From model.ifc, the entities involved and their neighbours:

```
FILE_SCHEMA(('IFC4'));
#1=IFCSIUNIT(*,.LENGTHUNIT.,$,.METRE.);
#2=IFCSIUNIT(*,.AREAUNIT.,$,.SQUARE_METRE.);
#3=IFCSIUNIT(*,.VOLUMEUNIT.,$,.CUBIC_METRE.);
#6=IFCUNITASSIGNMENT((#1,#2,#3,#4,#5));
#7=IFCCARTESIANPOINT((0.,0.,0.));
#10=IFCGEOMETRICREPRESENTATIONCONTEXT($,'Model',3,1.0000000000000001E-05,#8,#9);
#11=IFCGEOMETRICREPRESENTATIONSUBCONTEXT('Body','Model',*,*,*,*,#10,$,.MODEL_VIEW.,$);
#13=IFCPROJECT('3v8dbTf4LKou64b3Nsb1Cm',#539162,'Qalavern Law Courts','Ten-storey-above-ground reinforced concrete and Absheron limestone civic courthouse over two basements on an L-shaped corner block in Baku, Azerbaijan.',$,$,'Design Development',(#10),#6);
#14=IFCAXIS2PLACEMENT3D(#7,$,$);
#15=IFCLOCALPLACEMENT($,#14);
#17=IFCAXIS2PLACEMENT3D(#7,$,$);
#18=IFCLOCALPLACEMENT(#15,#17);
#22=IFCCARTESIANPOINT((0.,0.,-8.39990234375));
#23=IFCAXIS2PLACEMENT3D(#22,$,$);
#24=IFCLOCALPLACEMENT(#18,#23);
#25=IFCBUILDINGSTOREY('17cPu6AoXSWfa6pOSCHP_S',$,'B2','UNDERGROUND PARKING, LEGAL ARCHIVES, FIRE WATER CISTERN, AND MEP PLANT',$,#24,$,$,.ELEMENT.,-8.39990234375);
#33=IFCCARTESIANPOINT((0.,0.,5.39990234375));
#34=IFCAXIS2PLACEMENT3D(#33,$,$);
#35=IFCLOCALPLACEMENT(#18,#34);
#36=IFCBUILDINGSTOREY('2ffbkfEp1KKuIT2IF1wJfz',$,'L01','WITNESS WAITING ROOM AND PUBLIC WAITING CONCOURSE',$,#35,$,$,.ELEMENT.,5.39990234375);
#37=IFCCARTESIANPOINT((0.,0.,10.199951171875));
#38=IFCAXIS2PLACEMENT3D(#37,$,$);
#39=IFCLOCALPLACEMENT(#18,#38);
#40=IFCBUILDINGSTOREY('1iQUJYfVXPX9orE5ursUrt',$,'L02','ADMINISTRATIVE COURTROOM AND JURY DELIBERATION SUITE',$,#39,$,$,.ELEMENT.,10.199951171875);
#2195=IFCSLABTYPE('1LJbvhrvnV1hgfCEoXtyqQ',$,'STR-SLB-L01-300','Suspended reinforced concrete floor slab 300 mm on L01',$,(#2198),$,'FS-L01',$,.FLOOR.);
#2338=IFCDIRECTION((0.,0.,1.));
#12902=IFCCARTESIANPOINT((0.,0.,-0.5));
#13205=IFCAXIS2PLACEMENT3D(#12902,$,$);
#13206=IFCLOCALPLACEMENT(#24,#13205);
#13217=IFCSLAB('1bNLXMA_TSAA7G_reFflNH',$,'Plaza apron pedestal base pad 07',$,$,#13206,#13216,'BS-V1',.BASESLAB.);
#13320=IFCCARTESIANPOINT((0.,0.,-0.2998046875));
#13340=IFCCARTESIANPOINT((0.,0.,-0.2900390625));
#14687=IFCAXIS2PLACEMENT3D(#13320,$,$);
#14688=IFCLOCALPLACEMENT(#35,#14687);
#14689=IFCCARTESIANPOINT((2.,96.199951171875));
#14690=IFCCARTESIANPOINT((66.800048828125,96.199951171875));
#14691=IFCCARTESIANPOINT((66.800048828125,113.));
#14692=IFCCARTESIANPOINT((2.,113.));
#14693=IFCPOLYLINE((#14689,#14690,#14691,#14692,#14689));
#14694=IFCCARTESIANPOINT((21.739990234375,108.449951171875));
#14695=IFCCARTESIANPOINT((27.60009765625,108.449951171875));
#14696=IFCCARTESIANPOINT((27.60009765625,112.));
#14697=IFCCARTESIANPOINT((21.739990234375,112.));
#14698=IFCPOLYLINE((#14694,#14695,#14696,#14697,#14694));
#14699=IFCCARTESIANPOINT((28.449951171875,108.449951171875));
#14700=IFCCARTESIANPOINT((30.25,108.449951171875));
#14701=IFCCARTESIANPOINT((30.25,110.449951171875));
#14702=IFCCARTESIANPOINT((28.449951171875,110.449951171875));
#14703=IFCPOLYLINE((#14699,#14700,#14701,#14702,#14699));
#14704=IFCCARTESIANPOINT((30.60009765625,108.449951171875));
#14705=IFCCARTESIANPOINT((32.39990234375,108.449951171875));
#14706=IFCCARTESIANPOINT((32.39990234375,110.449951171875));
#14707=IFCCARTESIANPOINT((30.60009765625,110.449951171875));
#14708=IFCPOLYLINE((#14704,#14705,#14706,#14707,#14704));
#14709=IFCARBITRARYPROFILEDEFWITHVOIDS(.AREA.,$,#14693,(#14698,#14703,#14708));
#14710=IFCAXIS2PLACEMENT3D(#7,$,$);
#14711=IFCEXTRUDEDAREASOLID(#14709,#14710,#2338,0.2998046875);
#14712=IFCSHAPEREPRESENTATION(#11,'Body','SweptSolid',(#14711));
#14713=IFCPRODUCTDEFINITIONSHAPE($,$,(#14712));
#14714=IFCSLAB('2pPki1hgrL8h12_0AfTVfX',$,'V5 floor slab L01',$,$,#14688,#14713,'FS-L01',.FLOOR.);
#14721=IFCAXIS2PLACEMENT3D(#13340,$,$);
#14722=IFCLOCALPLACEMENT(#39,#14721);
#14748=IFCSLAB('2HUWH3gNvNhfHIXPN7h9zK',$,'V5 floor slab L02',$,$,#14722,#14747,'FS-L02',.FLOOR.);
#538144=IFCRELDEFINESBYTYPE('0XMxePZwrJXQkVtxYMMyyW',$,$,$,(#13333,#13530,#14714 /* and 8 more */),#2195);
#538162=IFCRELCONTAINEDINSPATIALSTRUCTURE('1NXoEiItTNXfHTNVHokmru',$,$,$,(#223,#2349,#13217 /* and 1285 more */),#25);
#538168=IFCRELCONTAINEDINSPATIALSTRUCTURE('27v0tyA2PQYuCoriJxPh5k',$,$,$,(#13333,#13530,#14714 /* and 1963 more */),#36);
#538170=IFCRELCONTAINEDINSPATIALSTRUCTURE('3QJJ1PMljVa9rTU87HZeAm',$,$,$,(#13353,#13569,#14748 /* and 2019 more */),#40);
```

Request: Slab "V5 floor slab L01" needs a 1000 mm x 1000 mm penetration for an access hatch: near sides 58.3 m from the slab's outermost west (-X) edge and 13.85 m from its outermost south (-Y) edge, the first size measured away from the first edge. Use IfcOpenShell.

```python
import numpy as np
import ifcopenshell
import ifcopenshell.api.feature
import ifcopenshell.api.geometry
import ifcopenshell.api.root
import ifcopenshell.geom
import ifcopenshell.util.placement
import ifcopenshell.util.representation
import ifcopenshell.util.shape
import ifcopenshell.util.unit

model = ifcopenshell.open("model.ifc")
unit_scale = ifcopenshell.util.unit.calculate_unit_scale(model)
settings = ifcopenshell.geom.settings()


def volume(element):
    """Net volume in cubic metres, openings subtracted."""
    shape = ifcopenshell.geom.create_shape(settings, element)
    return ifcopenshell.util.shape.get_volume(shape.geometry)


slab = model.by_guid("2pPki1hgrL8h12_0AfTVfX")
before = volume(slab)

# Extent in the slab's own axes, in metres. The edges named are its -X and -Y sides.
slab_shape = ifcopenshell.geom.create_shape(settings, slab)
vertices = ifcopenshell.util.shape.get_vertices(slab_shape.geometry)
x_min, y_min, bottom = vertices.min(axis=0)
top = vertices[:, 2].max()

opening = ifcopenshell.api.root.create_entity(model, ifc_class="IfcOpeningElement", name="Access hatch opening", predefined_type="OPENING")
context = ifcopenshell.util.representation.get_context(model, "Model", "Body", "MODEL_VIEW")
width, depth = 1, 1
outline = [(0.0, 0.0), (width, 0.0), (width, depth), (0.0, depth), (0.0, 0.0)]
# Overshoot both faces by 50 mm so the cut is clean.
shape = ifcopenshell.api.geometry.add_slab_representation(
    model, context=context, depth=top - bottom + 0.1, polyline=outline
)
ifcopenshell.api.geometry.assign_representation(model, product=opening, representation=shape)

matrix = ifcopenshell.util.placement.get_local_placement(slab.ObjectPlacement)
matrix[:, 3] = matrix @ np.append(np.array([x_min + 58.3, y_min + 13.85, bottom - 0.05]) / unit_scale, 1.0)
ifcopenshell.api.geometry.edit_object_placement(model, product=opening, matrix=matrix, is_si=False)
ifcopenshell.api.feature.add_feature(model, feature=opening, element=slab)

after = volume(slab)

print(f"slab volume {before:.3f} -> {after:.3f} m3")

model.write("model_edited.ifc")
```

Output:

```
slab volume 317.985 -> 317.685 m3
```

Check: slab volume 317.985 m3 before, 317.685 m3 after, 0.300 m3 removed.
